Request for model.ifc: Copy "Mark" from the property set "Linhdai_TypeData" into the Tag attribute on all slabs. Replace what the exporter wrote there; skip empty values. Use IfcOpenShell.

First a look at what the model holds.

```python
import ifcopenshell
import ifcopenshell.util.element

model = ifcopenshell.open("model.ifc")
print(model.schema)
slabs = model.by_type("IfcSlab")
print(len(slabs), "slabs")
for e in slabs[:8]:
    source = ifcopenshell.util.element.get_pset(e, "Linhdai_TypeData", "Mark")
    target = e.Tag
    print(e.id(), repr(source), repr(target), sep=" | ")
```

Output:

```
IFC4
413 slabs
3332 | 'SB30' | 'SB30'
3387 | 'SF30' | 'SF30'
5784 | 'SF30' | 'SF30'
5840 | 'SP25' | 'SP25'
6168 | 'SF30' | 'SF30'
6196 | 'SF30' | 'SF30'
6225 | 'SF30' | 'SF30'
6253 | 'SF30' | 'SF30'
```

```python
import ifcopenshell
import ifcopenshell.util.element

model = ifcopenshell.open("model.ifc")

count = 0
for e in model.by_type("IfcSlab"):
    value = ifcopenshell.util.element.get_pset(e, "Linhdai_TypeData", "Mark")
    current = e.Tag
    if not value or not value.strip() or current == value:
        continue
    e.Tag = value
    count += 1

print(count, "slabs updated")

model.write("model_edited.ifc")
```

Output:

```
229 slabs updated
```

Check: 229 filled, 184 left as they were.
